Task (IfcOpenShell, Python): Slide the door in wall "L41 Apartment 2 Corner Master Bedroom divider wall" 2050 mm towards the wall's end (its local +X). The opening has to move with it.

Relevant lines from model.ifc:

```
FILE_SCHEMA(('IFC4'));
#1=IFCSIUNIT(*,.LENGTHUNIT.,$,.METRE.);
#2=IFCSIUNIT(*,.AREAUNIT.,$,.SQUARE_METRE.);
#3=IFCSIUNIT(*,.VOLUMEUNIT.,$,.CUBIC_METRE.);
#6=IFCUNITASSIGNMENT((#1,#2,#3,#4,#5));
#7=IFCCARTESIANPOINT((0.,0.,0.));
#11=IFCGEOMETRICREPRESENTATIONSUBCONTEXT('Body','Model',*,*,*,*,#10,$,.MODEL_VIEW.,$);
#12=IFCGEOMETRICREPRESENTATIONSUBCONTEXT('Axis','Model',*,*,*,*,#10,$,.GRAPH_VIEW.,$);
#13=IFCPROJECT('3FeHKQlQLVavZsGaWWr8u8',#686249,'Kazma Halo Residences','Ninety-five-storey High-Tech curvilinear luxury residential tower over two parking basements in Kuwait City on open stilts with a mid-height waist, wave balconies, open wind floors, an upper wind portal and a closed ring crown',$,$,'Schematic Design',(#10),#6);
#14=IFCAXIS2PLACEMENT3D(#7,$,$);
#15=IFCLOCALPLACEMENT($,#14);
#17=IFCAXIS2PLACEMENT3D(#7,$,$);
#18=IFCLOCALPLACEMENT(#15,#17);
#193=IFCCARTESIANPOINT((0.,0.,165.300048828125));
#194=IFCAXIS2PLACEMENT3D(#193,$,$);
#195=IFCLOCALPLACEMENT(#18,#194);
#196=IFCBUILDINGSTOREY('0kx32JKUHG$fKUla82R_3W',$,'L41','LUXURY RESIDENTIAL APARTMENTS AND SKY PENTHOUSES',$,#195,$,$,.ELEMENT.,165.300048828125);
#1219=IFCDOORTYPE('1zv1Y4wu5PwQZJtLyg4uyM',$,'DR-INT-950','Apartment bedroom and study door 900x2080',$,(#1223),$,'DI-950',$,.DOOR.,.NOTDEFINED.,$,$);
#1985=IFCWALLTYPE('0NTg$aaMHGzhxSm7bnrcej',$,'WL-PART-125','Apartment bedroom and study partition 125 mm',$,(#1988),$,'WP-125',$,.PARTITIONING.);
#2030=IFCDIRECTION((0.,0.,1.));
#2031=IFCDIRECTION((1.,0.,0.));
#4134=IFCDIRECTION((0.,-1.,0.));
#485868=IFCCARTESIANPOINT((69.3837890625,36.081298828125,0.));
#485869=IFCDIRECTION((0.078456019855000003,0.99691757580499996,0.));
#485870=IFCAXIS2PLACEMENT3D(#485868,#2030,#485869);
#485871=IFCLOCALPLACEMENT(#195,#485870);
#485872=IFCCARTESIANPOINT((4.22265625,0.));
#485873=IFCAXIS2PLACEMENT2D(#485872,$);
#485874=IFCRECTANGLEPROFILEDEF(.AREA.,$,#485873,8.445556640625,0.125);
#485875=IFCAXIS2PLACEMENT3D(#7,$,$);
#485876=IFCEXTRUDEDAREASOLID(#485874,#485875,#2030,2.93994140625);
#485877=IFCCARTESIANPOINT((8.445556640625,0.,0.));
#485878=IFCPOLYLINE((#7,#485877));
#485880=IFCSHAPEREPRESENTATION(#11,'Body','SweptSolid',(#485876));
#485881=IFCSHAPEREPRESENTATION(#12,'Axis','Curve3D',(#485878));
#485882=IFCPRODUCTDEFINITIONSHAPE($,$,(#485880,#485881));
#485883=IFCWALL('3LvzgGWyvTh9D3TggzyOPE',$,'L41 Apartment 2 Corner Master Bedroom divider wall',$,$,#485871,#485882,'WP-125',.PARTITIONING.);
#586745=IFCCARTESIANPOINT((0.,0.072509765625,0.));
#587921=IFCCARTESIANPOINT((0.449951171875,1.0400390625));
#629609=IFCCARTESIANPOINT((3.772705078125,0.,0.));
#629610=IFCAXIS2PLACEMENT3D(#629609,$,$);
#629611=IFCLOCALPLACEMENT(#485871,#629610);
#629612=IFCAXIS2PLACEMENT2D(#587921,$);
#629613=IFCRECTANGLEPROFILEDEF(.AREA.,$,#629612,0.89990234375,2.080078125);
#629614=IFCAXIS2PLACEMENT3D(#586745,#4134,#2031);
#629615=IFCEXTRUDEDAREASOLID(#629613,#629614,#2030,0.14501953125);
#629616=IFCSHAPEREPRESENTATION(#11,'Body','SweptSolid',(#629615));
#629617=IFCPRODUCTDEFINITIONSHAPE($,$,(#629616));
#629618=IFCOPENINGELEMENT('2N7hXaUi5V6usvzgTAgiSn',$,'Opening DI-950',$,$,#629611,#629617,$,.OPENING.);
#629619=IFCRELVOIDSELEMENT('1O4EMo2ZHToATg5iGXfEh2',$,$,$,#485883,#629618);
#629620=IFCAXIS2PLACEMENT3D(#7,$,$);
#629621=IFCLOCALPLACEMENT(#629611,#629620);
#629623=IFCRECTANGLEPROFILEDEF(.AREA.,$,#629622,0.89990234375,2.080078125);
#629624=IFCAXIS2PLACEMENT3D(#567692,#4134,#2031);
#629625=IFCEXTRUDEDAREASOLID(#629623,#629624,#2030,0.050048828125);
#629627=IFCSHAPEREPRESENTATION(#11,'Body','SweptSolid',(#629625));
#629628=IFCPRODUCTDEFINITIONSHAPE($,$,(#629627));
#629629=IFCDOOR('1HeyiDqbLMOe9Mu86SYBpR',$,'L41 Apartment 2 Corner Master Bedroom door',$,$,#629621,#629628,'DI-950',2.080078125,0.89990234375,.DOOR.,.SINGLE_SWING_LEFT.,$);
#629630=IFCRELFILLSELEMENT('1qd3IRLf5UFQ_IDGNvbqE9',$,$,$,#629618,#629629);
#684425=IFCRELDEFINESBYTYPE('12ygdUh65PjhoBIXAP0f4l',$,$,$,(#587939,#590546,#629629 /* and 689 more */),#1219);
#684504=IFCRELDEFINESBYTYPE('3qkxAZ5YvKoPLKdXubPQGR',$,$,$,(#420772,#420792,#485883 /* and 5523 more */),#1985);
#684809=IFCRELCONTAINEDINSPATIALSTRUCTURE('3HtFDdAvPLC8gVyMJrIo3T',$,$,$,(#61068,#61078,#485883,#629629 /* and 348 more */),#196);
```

```python
import ifcopenshell
import ifcopenshell.api.geometry
import ifcopenshell.util.placement
import ifcopenshell.util.unit

model = ifcopenshell.open("model.ifc")
unit_scale = ifcopenshell.util.unit.calculate_unit_scale(model)

door = model.by_guid("1HeyiDqbLMOe9Mu86SYBpR")
opening = door.FillsVoids[0].RelatingOpeningElement
wall = opening.VoidsElements[0].RelatingBuildingElement

wall_matrix = ifcopenshell.util.placement.get_local_placement(wall.ObjectPlacement)
shift = wall_matrix[:3, 0] * 2.05 / unit_scale
before = ifcopenshell.util.placement.get_local_placement(door.ObjectPlacement)[:3, 3].copy()

# The door is placed relative to its opening, so it follows when the opening moves.
matrix = ifcopenshell.util.placement.get_local_placement(opening.ObjectPlacement)
matrix[:3, 3] += shift
ifcopenshell.api.geometry.edit_object_placement(
    model, product=opening, matrix=matrix, is_si=False, should_transform_children=True
)

after = ifcopenshell.util.placement.get_local_placement(door.ObjectPlacement)[:3, 3]
print("door moved by", (after - before).round(3) + 0.0)

model.write("model_edited.ifc")
```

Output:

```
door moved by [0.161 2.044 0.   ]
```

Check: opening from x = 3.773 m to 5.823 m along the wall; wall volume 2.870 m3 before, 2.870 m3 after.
